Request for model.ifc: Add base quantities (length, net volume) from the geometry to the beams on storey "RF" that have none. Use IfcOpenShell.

First a look at what the model holds.

```python
import ifcopenshell
import ifcopenshell.util.element
import ifcopenshell.util.unit

model = ifcopenshell.open("model.ifc")
print(model.schema)
for unit_type in ("LENGTHUNIT", "AREAUNIT", "VOLUMEUNIT"):
    print(unit_type, ifcopenshell.util.unit.calculate_unit_scale(model, unit_type))
storey = next(s for s in model.by_type("IfcBuildingStorey") if s.Name == "RF")
beams = [e for e in ifcopenshell.util.element.get_decomposition(storey) if e.is_a("IfcBeam")]
for e in sorted(beams, key=lambda e: e.id()):
    print(e.id(), e.is_a(), e.Name, list(ifcopenshell.util.element.get_psets(e, qtos_only=True)), sep=" | ")
```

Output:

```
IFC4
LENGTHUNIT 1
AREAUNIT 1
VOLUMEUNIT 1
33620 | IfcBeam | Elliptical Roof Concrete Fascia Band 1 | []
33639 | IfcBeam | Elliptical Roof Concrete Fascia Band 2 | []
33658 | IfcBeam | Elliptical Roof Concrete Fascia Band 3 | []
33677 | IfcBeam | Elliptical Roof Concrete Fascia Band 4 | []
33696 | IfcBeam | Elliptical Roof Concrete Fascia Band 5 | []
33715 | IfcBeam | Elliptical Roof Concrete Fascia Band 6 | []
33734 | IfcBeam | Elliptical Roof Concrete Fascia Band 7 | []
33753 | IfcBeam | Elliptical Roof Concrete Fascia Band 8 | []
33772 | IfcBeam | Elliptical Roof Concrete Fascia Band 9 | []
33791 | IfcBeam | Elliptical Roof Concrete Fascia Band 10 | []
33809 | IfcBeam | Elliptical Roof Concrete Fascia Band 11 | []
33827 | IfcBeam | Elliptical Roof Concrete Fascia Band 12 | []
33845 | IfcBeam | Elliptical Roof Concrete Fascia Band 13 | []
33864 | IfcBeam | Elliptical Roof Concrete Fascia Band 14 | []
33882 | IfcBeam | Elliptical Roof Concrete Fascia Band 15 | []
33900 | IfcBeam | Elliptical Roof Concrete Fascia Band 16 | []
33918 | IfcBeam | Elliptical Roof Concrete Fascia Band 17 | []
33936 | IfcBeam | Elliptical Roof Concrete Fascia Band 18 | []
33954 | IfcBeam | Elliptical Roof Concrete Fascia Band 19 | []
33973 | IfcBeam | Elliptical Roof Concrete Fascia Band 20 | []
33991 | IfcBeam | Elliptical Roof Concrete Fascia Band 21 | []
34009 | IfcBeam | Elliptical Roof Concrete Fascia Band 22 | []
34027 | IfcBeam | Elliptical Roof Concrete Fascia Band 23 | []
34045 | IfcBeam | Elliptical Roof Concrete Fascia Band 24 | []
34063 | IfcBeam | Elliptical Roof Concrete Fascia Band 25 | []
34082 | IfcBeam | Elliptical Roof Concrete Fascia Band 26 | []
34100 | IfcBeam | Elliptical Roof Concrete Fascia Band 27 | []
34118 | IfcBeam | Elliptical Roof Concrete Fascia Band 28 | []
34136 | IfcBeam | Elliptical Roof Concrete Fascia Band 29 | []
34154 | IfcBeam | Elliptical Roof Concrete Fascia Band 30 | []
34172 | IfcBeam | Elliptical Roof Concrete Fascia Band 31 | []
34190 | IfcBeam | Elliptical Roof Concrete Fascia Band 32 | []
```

```python
import ifcopenshell
import ifcopenshell.api.pset
import ifcopenshell.geom
import ifcopenshell.util.element
import ifcopenshell.util.shape
import ifcopenshell.util.unit

model = ifcopenshell.open("model.ifc")
unit_scale = ifcopenshell.util.unit.calculate_unit_scale(model)
volume_scale = ifcopenshell.util.unit.calculate_unit_scale(model, "VOLUMEUNIT")
settings = ifcopenshell.geom.settings()

storey = next(s for s in model.by_type("IfcBuildingStorey") if s.Name == "RF")
beams = [e for e in ifcopenshell.util.element.get_decomposition(storey) if e.is_a("IfcBeam")]

for e in sorted(beams, key=lambda e: e.id()):
    if ifcopenshell.util.element.get_psets(e, qtos_only=True, should_inherit=False):
        continue
    # Geometry comes back in metres, in the element's own axes.
    shape = ifcopenshell.geom.create_shape(settings, e)
    values = {
        "Length": ifcopenshell.util.shape.get_max_xyz(shape.geometry) / unit_scale,
        "NetVolume": ifcopenshell.util.shape.get_volume(shape.geometry) / volume_scale,
    }
    qto = ifcopenshell.api.pset.add_qto(model, product=e, name="Qto_BeamBaseQuantities")
    ifcopenshell.api.pset.edit_qto(model, qto=qto, properties=values)
    print(e.id(), {k: round(v, 3) for k, v in values.items()})

model.write("model-out.ifc")
```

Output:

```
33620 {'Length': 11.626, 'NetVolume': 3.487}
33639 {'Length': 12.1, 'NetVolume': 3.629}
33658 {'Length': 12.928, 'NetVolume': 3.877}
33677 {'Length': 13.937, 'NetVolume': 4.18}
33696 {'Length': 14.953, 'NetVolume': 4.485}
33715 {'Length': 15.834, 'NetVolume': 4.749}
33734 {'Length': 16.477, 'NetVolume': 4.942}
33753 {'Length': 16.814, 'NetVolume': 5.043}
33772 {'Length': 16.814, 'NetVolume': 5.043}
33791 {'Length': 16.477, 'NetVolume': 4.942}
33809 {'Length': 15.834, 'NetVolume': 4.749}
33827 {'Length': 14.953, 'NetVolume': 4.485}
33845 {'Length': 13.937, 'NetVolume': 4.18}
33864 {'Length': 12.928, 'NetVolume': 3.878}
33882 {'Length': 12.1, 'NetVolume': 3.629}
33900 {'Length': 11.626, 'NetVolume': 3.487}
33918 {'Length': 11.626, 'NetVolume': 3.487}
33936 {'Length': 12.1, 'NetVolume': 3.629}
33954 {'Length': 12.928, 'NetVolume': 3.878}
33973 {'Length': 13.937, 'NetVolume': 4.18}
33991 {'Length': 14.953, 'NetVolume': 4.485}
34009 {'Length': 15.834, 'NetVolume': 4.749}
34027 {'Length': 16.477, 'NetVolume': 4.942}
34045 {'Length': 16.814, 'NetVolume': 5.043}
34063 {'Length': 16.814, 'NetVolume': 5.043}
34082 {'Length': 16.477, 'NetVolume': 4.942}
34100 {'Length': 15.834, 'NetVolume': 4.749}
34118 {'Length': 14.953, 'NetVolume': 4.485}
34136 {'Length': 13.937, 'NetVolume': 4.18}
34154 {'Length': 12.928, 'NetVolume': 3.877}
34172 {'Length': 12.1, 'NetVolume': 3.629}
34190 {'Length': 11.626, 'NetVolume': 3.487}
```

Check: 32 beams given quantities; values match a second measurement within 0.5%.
